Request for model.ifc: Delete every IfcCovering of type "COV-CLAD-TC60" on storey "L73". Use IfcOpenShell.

First a look at what the model holds.

```python
import ifcopenshell
import ifcopenshell.util.element

model = ifcopenshell.open("model.ifc")
print(model.schema)
storey = next(s for s in model.by_type("IfcBuildingStorey") if s.Name == "L73")
coverings = [e for e in ifcopenshell.util.element.get_decomposition(storey) if e.is_a("IfcCovering")]
seen = {}
for e in coverings:
    element_type = ifcopenshell.util.element.get_type(e)
    name = element_type.Name if element_type not in (None, e) else None
    seen[name] = seen.get(name, 0) + 1
for name, count in sorted(seen.items(), key=str):
    print(count, "x", name)
```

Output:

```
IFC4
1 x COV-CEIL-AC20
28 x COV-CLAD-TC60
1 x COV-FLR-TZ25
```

```python
import ifcopenshell
import ifcopenshell.api.root
import ifcopenshell.util.element

model = ifcopenshell.open("model.ifc")

storey = next(s for s in model.by_type("IfcBuildingStorey") if s.Name == "L73")
coverings = [e for e in ifcopenshell.util.element.get_decomposition(storey) if e.is_a("IfcCovering")]
targets = [e for e in coverings if (t := ifcopenshell.util.element.get_type(e)) not in (None, e) and t.Name == "COV-CLAD-TC60"]

for e in targets:
    ifcopenshell.api.root.remove_product(model, product=e)
print(len(targets), "removed")

model.write("model_v2.ifc")
```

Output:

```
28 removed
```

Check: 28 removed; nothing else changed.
